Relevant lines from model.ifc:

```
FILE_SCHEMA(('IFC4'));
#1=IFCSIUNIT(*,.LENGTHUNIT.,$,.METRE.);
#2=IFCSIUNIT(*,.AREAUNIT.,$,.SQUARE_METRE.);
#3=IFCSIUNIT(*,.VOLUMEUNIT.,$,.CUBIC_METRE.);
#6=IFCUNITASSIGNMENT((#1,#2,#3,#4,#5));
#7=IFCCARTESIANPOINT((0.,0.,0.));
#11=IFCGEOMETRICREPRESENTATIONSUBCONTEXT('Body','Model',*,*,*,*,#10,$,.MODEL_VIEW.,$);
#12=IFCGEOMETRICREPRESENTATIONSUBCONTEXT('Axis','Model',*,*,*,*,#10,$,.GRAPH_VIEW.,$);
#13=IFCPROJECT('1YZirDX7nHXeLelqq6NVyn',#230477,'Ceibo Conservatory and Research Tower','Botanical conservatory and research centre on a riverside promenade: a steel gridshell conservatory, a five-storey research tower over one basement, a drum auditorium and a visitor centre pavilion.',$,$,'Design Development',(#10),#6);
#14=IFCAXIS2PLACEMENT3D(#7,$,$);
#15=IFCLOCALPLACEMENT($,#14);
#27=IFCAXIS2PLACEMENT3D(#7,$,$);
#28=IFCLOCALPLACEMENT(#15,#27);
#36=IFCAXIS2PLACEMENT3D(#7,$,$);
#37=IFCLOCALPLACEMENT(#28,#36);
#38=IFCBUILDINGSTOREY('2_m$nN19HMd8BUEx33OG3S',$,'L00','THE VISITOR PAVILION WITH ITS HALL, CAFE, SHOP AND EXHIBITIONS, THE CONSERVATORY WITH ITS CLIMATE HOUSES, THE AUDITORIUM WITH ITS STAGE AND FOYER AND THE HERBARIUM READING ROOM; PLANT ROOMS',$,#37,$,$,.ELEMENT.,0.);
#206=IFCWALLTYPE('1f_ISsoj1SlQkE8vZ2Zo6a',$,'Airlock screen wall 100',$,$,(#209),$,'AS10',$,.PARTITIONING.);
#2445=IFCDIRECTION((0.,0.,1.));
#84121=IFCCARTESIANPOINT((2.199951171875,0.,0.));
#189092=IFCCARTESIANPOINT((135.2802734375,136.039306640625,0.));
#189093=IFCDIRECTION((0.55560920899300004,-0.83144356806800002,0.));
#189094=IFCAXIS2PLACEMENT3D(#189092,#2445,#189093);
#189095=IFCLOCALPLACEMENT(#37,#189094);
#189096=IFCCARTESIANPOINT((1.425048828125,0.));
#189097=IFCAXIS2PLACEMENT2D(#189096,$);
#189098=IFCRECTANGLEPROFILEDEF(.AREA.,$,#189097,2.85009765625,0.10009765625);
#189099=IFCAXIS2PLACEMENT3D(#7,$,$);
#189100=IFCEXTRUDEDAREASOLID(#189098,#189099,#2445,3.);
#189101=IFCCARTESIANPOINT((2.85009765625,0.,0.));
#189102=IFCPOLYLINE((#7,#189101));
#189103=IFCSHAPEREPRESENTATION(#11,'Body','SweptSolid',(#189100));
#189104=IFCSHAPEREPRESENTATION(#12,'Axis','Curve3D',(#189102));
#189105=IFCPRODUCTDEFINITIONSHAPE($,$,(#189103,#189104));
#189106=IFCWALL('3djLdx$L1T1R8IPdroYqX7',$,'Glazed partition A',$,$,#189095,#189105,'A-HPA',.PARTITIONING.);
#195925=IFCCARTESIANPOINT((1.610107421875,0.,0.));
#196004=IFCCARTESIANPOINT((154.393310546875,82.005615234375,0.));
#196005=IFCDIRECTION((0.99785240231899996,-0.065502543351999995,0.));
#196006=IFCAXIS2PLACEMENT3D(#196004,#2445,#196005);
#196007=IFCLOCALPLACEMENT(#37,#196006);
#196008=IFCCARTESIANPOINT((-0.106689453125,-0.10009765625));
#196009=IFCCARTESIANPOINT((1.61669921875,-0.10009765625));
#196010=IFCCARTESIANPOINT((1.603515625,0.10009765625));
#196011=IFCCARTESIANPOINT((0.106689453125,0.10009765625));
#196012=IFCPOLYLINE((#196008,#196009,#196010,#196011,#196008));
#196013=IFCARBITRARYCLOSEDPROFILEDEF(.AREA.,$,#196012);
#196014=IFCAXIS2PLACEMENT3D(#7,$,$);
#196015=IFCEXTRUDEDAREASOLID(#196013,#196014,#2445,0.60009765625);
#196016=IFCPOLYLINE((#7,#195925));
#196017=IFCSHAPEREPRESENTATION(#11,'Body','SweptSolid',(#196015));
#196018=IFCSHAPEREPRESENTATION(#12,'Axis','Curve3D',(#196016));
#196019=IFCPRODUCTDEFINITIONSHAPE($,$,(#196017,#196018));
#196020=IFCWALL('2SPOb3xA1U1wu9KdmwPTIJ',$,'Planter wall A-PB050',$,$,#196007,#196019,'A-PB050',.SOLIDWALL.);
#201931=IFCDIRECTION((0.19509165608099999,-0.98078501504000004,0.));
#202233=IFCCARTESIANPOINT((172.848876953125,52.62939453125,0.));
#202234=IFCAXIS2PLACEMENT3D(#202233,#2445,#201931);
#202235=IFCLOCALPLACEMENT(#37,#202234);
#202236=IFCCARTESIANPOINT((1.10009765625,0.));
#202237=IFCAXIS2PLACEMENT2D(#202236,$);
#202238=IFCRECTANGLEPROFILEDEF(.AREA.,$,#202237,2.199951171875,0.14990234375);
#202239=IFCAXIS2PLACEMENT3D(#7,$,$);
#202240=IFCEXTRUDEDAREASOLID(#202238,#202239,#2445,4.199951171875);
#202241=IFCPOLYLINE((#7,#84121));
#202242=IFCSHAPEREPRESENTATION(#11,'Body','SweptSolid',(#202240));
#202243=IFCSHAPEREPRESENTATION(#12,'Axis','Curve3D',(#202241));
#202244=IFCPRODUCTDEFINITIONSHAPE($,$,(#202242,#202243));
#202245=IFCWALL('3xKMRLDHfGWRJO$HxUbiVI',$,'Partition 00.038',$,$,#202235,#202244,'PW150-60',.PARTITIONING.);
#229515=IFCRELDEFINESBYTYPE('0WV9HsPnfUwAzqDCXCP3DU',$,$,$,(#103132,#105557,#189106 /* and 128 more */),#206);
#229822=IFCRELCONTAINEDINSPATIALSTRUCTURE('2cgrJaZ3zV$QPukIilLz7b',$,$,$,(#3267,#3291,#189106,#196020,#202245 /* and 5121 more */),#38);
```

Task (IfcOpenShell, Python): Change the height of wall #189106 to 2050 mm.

```python
import ifcopenshell
import ifcopenshell.geom
import ifcopenshell.util.representation
import ifcopenshell.util.shape
import ifcopenshell.util.unit

model = ifcopenshell.open("model.ifc")
unit_scale = ifcopenshell.util.unit.calculate_unit_scale(model)
settings = ifcopenshell.geom.settings()


def volume(element):
    """Net volume in cubic metres, openings subtracted."""
    shape = ifcopenshell.geom.create_shape(settings, element)
    return ifcopenshell.util.shape.get_volume(shape.geometry)


wall = model.by_guid("3djLdx$L1T1R8IPdroYqX7")
before = volume(wall)

body = ifcopenshell.util.representation.get_representation(wall, "Model", "Body")
solid = body.Items[0]
old_height = solid.Depth
solid.Depth = 2.05 / unit_scale
after = volume(wall)

print(f"height {old_height:g} -> {solid.Depth:g}, volume {before:.3f} -> {after:.3f} m3")

model.write("model_rev.ifc")
```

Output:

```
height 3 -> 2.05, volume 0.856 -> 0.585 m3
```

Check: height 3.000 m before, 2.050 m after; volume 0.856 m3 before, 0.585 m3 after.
